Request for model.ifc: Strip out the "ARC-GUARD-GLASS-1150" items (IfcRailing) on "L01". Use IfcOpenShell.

First a look at what the model holds.

```python
import ifcopenshell
import ifcopenshell.util.element

model = ifcopenshell.open("model.ifc")
print(model.schema)
storey = next(s for s in model.by_type("IfcBuildingStorey") if s.Name == "L01")
railings = [e for e in ifcopenshell.util.element.get_decomposition(storey) if e.is_a("IfcRailing")]
seen = {}
for e in railings:
    element_type = ifcopenshell.util.element.get_type(e)
    name = element_type.Name if element_type not in (None, e) else None
    seen[name] = seen.get(name, 0) + 1
for name, count in sorted(seen.items(), key=str):
    print(count, "x", name)
```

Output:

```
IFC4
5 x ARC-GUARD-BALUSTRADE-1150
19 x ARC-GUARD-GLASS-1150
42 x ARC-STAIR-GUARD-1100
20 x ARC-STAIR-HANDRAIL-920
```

```python
import ifcopenshell
import ifcopenshell.api.root
import ifcopenshell.util.element

model = ifcopenshell.open("model.ifc")

storey = next(s for s in model.by_type("IfcBuildingStorey") if s.Name == "L01")
railings = [e for e in ifcopenshell.util.element.get_decomposition(storey) if e.is_a("IfcRailing")]
targets = [e for e in railings if (t := ifcopenshell.util.element.get_type(e)) not in (None, e) and t.Name == "ARC-GUARD-GLASS-1150"]

for e in targets:
    ifcopenshell.api.root.remove_product(model, product=e)
print(len(targets), "removed")

model.write("model_v2.ifc")
```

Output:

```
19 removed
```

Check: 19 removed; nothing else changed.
